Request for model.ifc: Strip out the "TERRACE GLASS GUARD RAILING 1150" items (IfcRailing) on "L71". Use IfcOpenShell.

First a look at what the model holds.

```python
import ifcopenshell
import ifcopenshell.util.element

model = ifcopenshell.open("model.ifc")
print(model.schema)
storey = next(s for s in model.by_type("IfcBuildingStorey") if s.Name == "L71")
railings = [e for e in ifcopenshell.util.element.get_decomposition(storey) if e.is_a("IfcRailing")]
seen = {}
for e in railings:
    element_type = ifcopenshell.util.element.get_type(e)
    name = element_type.Name if element_type not in (None, e) else None
    seen[name] = seen.get(name, 0) + 1
for name, count in sorted(seen.items(), key=str):
    print(count, "x", name)
```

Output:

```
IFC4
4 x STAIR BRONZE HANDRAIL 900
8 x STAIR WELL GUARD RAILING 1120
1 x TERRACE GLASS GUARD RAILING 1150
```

```python
import ifcopenshell
import ifcopenshell.api.root
import ifcopenshell.util.element

model = ifcopenshell.open("model.ifc")

storey = next(s for s in model.by_type("IfcBuildingStorey") if s.Name == "L71")
railings = [e for e in ifcopenshell.util.element.get_decomposition(storey) if e.is_a("IfcRailing")]
targets = [e for e in railings if (t := ifcopenshell.util.element.get_type(e)) not in (None, e) and t.Name == "TERRACE GLASS GUARD RAILING 1150"]

for e in targets:
    ifcopenshell.api.root.remove_product(model, product=e)
print(len(targets), "removed")

model.write("model_rev.ifc")
```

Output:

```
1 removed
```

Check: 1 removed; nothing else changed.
